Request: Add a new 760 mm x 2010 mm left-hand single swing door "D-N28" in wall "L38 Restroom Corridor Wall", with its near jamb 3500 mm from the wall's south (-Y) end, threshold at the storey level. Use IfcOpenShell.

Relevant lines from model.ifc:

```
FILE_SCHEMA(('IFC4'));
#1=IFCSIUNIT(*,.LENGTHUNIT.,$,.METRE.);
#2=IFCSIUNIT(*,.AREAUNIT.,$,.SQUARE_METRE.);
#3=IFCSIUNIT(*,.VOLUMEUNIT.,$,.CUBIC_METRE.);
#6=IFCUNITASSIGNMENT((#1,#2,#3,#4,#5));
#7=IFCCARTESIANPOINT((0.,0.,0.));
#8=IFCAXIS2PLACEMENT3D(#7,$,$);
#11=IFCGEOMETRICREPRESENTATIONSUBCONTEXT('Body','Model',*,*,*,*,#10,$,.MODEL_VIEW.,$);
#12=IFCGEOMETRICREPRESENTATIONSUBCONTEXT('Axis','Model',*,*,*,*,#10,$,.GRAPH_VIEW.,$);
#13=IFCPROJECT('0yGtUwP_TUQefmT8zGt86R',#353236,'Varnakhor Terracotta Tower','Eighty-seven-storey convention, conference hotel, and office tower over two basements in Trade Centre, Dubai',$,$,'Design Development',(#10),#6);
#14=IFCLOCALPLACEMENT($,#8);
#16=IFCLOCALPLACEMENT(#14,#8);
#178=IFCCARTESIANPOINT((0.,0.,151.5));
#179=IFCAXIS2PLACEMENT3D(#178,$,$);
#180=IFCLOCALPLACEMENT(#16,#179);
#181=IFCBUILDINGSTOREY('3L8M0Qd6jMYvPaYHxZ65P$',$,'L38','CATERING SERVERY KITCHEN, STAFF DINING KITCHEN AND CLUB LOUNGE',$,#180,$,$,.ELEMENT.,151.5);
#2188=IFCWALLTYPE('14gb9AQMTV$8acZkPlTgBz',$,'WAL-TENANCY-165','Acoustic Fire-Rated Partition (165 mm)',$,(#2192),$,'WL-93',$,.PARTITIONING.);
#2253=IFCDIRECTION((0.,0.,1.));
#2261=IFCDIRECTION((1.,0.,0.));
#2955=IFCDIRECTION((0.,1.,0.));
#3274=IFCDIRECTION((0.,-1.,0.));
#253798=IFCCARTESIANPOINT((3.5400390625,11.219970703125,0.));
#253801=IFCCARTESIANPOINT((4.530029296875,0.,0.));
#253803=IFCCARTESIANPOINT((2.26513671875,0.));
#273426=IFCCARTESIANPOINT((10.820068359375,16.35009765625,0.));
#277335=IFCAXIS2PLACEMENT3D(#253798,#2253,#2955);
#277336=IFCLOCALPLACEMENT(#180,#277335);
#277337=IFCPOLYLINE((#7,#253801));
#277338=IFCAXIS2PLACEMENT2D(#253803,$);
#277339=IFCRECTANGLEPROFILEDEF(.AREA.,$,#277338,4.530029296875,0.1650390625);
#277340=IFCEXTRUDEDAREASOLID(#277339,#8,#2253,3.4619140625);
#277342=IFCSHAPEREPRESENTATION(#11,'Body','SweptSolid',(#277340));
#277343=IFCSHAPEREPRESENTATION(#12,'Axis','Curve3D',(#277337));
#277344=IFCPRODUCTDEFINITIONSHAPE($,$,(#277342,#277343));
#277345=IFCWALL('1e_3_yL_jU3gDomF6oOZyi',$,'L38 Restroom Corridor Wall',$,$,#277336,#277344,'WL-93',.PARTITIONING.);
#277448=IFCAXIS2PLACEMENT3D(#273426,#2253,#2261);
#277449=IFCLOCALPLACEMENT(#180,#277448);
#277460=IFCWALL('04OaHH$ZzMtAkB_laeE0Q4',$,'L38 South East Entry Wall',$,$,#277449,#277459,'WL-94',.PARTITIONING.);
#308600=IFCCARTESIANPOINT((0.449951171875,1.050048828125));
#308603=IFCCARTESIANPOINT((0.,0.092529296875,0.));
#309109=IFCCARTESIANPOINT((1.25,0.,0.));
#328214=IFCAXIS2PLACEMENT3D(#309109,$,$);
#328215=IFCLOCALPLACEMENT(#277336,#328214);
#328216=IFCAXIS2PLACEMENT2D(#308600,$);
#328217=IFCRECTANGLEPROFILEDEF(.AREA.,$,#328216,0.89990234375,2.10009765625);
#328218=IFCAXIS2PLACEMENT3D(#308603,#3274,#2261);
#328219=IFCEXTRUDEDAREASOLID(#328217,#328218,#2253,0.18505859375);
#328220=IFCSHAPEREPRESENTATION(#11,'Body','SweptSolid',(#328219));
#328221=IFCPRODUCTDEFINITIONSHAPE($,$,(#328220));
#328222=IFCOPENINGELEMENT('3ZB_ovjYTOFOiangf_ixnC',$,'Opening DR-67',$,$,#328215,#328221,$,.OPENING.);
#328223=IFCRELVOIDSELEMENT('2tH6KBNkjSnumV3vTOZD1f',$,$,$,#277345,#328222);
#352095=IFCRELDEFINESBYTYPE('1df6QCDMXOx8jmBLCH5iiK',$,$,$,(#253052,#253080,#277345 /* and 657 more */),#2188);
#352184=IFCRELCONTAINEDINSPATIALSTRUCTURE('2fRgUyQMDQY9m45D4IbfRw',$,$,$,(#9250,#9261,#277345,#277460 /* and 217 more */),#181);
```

```python
import numpy as np
import ifcopenshell
import ifcopenshell.api.feature
import ifcopenshell.api.geometry
import ifcopenshell.api.root
import ifcopenshell.api.spatial
import ifcopenshell.geom
import ifcopenshell.util.element
import ifcopenshell.util.placement
import ifcopenshell.util.representation
import ifcopenshell.util.shape
import ifcopenshell.util.unit

model = ifcopenshell.open("model.ifc")
unit_scale = ifcopenshell.util.unit.calculate_unit_scale(model)
settings = ifcopenshell.geom.settings()


def volume(element):
    """Net volume in cubic metres, openings subtracted."""
    shape = ifcopenshell.geom.create_shape(settings, element)
    return ifcopenshell.util.shape.get_volume(shape.geometry)


wall = model.by_guid("1e_3_yL_jU3gDomF6oOZyi")
storey = ifcopenshell.util.element.get_container(wall, ifc_class="IfcBuildingStorey")
context = ifcopenshell.util.representation.get_context(model, "Model", "Body", "MODEL_VIEW")
before = volume(wall)

width, height, from_end, sill = 0.76, 2.01, 3.5, 0.0  # metres

# The wall runs along its own X axis, and the end named is its -X end.
wall_shape = ifcopenshell.geom.create_shape(settings, wall)
x, y, z = ifcopenshell.util.shape.get_vertices(wall_shape.geometry).T
start = x.min() + from_end
face, thickness = float(y.min()), float(y.max() - y.min())
wall_matrix = ifcopenshell.util.placement.get_local_placement(wall.ObjectPlacement)
level = ifcopenshell.util.placement.get_local_placement(storey.ObjectPlacement)[2, 3]


def in_wall(x, y):
    """Placement at x, y metres in the wall's axes, at sill height."""
    matrix = wall_matrix.copy()
    matrix[:, 3] = wall_matrix @ np.array([x / unit_scale, y / unit_scale, 0.0, 1.0])
    matrix[2, 3] = level + sill / unit_scale
    return matrix


# Opening: a box that overshoots both wall faces by 50 mm.
opening = ifcopenshell.api.root.create_entity(model, ifc_class="IfcOpeningElement", predefined_type="OPENING")
box = ifcopenshell.api.geometry.add_wall_representation(
    model, context=context, length=width, height=height, thickness=thickness + 0.1
)
ifcopenshell.api.geometry.assign_representation(model, product=opening, representation=box)
ifcopenshell.api.geometry.edit_object_placement(model, product=opening, matrix=in_wall(start, face - 0.05), is_si=False)
ifcopenshell.api.feature.add_feature(model, feature=opening, element=wall)

door = ifcopenshell.api.root.create_entity(model, ifc_class="IfcDoor", name="D-N28", predefined_type="DOOR")
door.OverallWidth, door.OverallHeight = width / unit_scale, height / unit_scale
door.OperationType = "SINGLE_SWING_LEFT"
body = ifcopenshell.api.geometry.add_door_representation(
    model,
    context=context,
    overall_width=door.OverallWidth,
    overall_height=door.OverallHeight,
    operation_type="SINGLE_SWING_LEFT",
    lining_properties={"LiningDepth": thickness / unit_scale, "ThresholdDepth": thickness / unit_scale},
)
ifcopenshell.api.geometry.assign_representation(model, product=door, representation=body)
ifcopenshell.api.spatial.assign_container(model, products=[door], relating_structure=storey)
ifcopenshell.api.feature.add_filling(model, opening=opening, element=door)

# The lining spans the wall, so the door starts at the wall face.
ifcopenshell.api.geometry.edit_object_placement(model, product=door, matrix=in_wall(start, face), is_si=False)

after = volume(wall)

print(f"wall volume {before:.3f} -> {after:.3f} m3")

model.write("model_rev.ifc")
```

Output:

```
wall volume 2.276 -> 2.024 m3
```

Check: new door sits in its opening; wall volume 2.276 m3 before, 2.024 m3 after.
